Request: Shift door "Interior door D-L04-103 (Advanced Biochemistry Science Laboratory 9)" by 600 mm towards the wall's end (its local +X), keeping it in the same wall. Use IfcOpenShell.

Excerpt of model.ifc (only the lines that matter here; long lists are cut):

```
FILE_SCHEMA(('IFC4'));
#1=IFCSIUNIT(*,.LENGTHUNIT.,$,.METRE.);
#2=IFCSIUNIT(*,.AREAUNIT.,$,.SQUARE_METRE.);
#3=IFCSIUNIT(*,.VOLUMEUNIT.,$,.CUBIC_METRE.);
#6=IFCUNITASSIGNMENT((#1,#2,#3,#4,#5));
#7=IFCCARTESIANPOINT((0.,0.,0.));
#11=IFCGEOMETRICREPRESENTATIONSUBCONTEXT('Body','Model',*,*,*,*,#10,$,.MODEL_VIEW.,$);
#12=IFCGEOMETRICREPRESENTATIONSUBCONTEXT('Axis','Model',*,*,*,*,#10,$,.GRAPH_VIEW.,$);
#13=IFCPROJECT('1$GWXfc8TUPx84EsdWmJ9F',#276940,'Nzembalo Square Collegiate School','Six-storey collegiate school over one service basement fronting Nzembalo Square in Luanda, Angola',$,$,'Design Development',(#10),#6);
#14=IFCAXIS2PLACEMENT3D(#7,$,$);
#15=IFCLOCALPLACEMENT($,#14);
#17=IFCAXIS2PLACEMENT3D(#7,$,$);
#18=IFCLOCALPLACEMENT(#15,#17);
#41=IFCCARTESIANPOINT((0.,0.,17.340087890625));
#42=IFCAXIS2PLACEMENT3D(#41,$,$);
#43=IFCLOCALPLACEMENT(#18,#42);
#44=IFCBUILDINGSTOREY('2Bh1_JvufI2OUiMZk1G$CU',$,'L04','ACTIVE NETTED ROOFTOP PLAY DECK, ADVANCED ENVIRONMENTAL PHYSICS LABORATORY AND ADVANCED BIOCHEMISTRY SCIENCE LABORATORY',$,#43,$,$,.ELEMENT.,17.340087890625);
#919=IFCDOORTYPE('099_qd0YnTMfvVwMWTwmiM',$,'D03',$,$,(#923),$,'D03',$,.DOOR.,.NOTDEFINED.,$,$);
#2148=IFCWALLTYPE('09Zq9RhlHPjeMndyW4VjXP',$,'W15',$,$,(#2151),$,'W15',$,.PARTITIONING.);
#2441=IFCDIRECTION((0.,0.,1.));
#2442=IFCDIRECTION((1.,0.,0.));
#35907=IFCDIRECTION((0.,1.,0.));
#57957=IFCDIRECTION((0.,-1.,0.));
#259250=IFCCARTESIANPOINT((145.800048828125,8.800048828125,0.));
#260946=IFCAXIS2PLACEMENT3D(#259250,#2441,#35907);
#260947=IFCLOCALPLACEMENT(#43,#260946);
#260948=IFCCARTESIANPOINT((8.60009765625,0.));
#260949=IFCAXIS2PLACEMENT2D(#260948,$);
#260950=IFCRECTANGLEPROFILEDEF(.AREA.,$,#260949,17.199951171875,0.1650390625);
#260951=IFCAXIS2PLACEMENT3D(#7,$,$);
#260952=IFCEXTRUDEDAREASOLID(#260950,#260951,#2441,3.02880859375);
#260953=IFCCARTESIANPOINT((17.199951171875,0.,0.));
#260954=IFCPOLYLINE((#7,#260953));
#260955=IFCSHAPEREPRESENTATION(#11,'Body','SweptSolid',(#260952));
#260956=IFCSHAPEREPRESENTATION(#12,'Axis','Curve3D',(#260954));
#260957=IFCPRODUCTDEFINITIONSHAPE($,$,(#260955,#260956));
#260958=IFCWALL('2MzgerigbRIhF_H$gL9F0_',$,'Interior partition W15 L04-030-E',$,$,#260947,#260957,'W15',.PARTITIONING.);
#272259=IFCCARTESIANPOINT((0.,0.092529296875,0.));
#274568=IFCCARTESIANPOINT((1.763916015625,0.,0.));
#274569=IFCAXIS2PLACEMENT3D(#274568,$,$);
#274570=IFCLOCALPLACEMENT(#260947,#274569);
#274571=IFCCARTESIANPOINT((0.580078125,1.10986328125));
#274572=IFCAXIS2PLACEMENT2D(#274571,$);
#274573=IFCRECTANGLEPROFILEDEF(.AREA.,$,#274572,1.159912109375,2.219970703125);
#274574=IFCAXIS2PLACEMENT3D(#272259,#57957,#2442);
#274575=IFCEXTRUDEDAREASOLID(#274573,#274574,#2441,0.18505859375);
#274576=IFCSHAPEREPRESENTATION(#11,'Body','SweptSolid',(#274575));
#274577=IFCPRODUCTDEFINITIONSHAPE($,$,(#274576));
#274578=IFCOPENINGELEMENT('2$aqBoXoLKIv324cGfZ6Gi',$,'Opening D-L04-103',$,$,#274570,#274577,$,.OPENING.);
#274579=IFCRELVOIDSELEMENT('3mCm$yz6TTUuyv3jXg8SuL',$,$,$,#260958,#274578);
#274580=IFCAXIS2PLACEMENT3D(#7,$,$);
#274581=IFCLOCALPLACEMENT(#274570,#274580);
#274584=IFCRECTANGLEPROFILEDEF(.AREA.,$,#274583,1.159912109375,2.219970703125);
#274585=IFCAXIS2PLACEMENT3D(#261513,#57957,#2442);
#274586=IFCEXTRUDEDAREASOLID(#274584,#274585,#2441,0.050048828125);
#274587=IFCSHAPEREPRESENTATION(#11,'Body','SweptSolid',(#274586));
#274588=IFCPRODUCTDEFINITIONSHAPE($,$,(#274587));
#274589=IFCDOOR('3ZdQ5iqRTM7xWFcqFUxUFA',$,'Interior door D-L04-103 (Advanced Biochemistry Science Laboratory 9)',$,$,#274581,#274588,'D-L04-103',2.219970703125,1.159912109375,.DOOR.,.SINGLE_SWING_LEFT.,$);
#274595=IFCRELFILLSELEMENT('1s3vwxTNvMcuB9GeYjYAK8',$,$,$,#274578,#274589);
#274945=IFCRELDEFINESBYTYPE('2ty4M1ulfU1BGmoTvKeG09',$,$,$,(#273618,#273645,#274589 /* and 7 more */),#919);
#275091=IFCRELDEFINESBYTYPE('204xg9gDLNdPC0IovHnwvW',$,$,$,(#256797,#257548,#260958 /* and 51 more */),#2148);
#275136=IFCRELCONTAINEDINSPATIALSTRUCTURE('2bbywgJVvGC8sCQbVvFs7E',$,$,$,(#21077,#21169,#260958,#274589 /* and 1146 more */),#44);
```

```python
import ifcopenshell
import ifcopenshell.api.geometry
import ifcopenshell.util.placement

model = ifcopenshell.open("model.ifc")

door = model.by_id(274589)
opening = door.FillsVoids[0].RelatingOpeningElement
wall = opening.VoidsElements[0].RelatingBuildingElement

wall_matrix = ifcopenshell.util.placement.get_local_placement(wall.ObjectPlacement)
shift = wall_matrix[:3, 0] * 0.6
before = ifcopenshell.util.placement.get_local_placement(door.ObjectPlacement)[:3, 3].copy()

# The door is placed relative to its opening, so it follows when the opening moves.
matrix = ifcopenshell.util.placement.get_local_placement(opening.ObjectPlacement)
matrix[:3, 3] += shift
ifcopenshell.api.geometry.edit_object_placement(
    model, product=opening, matrix=matrix, is_si=False, should_transform_children=True
)

after = ifcopenshell.util.placement.get_local_placement(door.ObjectPlacement)[:3, 3]
print("door moved by", (after - before).round(3) + 0.0)

model.write("model-out.ifc")
```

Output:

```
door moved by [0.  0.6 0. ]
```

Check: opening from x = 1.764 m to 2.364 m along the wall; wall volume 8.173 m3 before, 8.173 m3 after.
